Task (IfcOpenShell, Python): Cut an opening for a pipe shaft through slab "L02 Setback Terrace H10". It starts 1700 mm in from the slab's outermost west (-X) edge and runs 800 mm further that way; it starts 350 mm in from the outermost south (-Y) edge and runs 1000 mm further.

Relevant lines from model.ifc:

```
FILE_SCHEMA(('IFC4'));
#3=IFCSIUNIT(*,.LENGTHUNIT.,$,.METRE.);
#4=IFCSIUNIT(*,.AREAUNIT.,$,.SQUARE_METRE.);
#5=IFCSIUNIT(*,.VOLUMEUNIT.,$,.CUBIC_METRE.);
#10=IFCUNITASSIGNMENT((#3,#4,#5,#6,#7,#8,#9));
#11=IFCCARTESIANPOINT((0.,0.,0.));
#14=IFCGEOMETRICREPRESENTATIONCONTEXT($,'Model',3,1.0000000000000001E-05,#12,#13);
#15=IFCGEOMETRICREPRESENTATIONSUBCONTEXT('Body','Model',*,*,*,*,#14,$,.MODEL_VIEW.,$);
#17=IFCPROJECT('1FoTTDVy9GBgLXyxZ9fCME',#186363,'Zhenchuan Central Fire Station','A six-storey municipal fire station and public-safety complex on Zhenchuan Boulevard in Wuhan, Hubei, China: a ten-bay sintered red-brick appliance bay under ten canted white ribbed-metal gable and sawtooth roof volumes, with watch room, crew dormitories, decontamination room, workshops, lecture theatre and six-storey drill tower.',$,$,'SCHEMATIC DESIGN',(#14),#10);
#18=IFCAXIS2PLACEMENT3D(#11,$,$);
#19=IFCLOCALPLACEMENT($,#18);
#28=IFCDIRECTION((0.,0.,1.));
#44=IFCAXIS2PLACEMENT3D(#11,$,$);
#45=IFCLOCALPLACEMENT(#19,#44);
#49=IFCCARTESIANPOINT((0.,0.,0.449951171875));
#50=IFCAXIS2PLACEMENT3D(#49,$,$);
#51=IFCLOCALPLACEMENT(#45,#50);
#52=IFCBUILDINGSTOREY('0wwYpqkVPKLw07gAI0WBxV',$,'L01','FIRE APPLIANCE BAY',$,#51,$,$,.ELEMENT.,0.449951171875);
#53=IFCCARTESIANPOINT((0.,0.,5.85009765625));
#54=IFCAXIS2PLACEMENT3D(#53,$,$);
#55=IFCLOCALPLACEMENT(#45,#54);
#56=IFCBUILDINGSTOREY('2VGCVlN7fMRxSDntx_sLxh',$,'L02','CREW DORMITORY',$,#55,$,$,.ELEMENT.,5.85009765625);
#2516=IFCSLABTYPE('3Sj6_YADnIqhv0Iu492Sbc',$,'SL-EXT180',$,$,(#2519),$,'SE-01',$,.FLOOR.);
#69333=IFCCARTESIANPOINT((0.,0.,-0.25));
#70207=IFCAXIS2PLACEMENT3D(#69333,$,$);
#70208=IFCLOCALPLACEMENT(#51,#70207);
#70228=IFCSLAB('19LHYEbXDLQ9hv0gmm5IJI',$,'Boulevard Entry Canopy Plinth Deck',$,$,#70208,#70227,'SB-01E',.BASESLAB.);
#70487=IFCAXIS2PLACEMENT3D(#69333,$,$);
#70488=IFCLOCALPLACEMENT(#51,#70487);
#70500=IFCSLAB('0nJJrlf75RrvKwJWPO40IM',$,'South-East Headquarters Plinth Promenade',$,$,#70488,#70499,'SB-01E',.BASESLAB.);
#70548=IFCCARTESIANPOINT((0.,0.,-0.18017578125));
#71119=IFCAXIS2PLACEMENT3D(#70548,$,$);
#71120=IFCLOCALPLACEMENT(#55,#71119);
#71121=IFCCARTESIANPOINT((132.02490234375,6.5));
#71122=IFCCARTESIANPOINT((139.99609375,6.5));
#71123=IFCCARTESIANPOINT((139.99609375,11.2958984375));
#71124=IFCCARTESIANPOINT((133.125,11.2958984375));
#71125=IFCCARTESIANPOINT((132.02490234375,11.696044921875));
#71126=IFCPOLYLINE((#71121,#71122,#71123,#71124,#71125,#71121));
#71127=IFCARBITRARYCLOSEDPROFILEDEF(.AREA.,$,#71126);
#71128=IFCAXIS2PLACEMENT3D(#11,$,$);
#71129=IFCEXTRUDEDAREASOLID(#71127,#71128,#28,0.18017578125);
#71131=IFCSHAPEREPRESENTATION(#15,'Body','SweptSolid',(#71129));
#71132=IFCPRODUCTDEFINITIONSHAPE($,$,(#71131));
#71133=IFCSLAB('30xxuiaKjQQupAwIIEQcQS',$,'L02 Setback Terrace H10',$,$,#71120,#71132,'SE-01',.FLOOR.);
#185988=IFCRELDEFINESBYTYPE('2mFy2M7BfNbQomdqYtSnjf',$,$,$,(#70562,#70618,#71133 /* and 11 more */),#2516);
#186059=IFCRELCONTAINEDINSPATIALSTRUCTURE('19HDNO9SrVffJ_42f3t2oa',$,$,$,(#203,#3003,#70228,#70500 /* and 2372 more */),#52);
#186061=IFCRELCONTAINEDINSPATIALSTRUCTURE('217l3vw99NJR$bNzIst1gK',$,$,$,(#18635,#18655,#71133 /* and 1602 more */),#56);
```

```python
import numpy as np
import ifcopenshell
import ifcopenshell.api.feature
import ifcopenshell.api.geometry
import ifcopenshell.api.root
import ifcopenshell.geom
import ifcopenshell.util.placement
import ifcopenshell.util.representation
import ifcopenshell.util.shape
import ifcopenshell.util.unit

model = ifcopenshell.open("model.ifc")
unit_scale = ifcopenshell.util.unit.calculate_unit_scale(model)
settings = ifcopenshell.geom.settings()


def volume(element):
    """Net volume in cubic metres, openings subtracted."""
    shape = ifcopenshell.geom.create_shape(settings, element)
    return ifcopenshell.util.shape.get_volume(shape.geometry)


slab = model.by_id(71133)
before = volume(slab)

# Extent in the slab's own axes, in metres. The edges named are its -X and -Y sides.
slab_shape = ifcopenshell.geom.create_shape(settings, slab)
vertices = ifcopenshell.util.shape.get_vertices(slab_shape.geometry)
x_min, y_min, bottom = vertices.min(axis=0)
top = vertices[:, 2].max()

opening = ifcopenshell.api.root.create_entity(model, ifc_class="IfcOpeningElement", name="Pipe shaft opening", predefined_type="OPENING")
context = ifcopenshell.util.representation.get_context(model, "Model", "Body", "MODEL_VIEW")
width, depth = 0.8, 1
outline = [(0.0, 0.0), (width, 0.0), (width, depth), (0.0, depth), (0.0, 0.0)]
# Overshoot both faces by 50 mm so the cut is clean.
shape = ifcopenshell.api.geometry.add_slab_representation(
    model, context=context, depth=top - bottom + 0.1, polyline=outline
)
ifcopenshell.api.geometry.assign_representation(model, product=opening, representation=shape)

matrix = ifcopenshell.util.placement.get_local_placement(slab.ObjectPlacement)
matrix[:, 3] = matrix @ np.append(np.array([x_min + 1.7, y_min + 0.35, bottom - 0.05]) / unit_scale, 1.0)
ifcopenshell.api.geometry.edit_object_placement(model, product=opening, matrix=matrix, is_si=False)
ifcopenshell.api.feature.add_feature(model, feature=opening, element=slab)

after = volume(slab)

print(f"slab volume {before:.3f} -> {after:.3f} m3")

model.write("model_v2.ifc")
```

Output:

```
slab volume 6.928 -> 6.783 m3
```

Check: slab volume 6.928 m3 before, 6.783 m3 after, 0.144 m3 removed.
